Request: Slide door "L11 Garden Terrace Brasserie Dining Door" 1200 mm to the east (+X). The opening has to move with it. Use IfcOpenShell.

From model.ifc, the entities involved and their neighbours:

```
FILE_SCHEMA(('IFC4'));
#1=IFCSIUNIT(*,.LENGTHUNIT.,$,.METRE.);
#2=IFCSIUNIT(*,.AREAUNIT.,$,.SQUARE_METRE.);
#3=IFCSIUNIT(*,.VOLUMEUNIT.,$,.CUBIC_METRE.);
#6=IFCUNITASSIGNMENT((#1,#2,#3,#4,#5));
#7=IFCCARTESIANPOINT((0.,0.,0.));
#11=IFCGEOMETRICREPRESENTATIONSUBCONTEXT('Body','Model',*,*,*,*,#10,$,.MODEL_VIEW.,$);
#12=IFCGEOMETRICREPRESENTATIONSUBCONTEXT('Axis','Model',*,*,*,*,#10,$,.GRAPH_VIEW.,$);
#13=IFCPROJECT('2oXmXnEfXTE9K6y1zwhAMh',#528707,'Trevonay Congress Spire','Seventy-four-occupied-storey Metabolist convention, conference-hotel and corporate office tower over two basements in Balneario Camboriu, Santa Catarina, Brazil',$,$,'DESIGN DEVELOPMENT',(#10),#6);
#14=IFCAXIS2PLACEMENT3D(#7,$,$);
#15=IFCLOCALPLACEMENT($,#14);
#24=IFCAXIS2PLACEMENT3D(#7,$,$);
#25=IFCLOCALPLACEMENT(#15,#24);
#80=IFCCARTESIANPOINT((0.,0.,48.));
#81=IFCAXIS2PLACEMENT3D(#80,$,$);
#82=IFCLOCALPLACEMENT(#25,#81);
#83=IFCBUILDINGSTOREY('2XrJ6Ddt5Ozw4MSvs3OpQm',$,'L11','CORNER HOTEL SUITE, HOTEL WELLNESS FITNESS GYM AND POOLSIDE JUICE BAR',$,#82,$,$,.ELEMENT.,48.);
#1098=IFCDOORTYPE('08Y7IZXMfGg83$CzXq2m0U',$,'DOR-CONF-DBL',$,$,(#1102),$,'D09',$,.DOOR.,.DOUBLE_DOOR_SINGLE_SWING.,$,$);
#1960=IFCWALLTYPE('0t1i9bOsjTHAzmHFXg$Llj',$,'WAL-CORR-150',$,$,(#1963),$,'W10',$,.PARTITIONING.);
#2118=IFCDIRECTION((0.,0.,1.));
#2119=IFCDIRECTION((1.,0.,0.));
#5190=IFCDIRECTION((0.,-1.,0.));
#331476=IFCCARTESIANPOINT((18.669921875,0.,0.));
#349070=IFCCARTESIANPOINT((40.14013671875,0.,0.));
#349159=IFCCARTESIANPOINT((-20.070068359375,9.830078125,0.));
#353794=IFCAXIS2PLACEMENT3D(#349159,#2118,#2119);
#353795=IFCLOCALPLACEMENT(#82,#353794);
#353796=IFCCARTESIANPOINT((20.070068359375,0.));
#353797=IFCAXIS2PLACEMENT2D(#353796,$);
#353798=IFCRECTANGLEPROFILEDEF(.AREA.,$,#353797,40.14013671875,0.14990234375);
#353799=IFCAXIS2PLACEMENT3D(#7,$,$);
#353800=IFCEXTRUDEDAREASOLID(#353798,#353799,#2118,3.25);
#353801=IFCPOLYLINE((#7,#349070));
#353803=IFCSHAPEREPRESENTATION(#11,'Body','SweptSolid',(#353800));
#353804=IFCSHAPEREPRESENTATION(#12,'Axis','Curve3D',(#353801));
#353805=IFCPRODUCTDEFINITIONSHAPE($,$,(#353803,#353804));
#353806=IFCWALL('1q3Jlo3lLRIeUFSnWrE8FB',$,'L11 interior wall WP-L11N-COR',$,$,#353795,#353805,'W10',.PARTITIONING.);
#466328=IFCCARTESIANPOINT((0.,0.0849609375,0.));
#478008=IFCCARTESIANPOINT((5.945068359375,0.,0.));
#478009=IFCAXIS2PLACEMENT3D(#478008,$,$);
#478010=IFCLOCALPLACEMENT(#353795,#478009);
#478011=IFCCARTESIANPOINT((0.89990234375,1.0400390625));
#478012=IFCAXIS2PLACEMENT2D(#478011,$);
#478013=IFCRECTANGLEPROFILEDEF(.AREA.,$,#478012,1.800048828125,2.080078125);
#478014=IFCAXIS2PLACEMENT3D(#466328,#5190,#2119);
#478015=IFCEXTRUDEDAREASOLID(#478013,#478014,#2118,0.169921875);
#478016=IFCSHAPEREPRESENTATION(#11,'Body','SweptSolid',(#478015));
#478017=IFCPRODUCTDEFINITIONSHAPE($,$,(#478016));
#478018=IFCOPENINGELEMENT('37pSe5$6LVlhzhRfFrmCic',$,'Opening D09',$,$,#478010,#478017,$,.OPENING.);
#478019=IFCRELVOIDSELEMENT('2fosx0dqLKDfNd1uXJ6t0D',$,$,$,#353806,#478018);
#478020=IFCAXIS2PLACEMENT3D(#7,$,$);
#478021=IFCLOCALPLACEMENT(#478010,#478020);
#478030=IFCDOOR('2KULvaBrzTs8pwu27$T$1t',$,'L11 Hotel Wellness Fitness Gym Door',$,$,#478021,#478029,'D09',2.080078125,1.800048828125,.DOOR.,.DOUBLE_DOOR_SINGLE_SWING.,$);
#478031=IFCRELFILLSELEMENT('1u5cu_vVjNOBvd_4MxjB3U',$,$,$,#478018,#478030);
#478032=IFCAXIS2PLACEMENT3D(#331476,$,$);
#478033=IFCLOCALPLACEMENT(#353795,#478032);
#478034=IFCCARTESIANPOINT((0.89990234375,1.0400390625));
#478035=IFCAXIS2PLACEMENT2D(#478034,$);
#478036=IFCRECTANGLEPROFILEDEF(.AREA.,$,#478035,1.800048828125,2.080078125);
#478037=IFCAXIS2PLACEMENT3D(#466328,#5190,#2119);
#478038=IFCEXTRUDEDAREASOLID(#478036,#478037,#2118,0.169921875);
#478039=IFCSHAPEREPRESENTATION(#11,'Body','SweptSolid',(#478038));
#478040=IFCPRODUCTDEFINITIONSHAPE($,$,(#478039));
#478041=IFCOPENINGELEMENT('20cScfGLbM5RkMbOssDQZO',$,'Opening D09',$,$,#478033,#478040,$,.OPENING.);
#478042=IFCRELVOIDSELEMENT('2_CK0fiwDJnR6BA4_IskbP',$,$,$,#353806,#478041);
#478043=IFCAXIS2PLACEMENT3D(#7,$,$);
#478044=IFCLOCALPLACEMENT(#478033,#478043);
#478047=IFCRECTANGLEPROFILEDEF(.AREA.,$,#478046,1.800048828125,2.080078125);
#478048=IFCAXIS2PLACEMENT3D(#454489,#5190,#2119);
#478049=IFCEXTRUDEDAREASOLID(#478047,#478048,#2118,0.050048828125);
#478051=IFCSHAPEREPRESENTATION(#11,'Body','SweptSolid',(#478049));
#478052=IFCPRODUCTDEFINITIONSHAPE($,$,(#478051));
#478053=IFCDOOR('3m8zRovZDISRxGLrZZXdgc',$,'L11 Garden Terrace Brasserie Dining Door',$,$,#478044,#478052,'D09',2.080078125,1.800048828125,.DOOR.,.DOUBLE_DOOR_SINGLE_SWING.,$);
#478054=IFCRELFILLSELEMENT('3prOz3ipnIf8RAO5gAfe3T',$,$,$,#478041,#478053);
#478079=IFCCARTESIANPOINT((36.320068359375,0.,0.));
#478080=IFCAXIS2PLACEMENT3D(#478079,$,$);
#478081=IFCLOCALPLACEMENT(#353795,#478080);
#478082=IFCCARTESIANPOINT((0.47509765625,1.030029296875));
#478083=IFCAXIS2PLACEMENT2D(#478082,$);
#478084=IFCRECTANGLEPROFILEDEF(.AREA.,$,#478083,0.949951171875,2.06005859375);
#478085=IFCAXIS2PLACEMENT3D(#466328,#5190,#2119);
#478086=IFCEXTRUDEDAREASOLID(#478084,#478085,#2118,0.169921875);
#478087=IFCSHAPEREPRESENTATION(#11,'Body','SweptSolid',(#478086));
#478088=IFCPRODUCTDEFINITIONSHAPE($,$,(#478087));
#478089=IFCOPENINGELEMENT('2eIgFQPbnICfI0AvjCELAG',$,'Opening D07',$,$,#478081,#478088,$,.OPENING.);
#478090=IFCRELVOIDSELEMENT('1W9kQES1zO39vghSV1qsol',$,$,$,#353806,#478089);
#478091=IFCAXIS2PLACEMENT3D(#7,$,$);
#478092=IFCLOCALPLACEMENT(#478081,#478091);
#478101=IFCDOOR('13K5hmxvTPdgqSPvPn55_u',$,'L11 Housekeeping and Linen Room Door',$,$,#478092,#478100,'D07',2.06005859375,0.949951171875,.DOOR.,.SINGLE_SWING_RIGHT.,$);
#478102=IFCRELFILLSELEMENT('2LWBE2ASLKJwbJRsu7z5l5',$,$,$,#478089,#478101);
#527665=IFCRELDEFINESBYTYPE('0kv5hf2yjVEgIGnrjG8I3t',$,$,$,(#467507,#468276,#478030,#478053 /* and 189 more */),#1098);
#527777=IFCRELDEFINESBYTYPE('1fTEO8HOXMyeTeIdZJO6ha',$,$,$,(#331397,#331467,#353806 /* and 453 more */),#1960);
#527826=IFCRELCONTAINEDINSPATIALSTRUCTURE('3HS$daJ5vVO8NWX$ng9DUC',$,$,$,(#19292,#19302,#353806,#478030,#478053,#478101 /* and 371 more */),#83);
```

```python
import ifcopenshell
import ifcopenshell.api.geometry
import ifcopenshell.util.placement

model = ifcopenshell.open("model.ifc")

door = model.by_guid("3m8zRovZDISRxGLrZZXdgc")
opening = door.FillsVoids[0].RelatingOpeningElement
wall = opening.VoidsElements[0].RelatingBuildingElement

wall_matrix = ifcopenshell.util.placement.get_local_placement(wall.ObjectPlacement)
shift = wall_matrix[:3, 0] * 1.2
before = ifcopenshell.util.placement.get_local_placement(door.ObjectPlacement)[:3, 3].copy()

# The door is placed relative to its opening, so it follows when the opening moves.
matrix = ifcopenshell.util.placement.get_local_placement(opening.ObjectPlacement)
matrix[:3, 3] += shift
ifcopenshell.api.geometry.edit_object_placement(
    model, product=opening, matrix=matrix, is_si=False, should_transform_children=True
)

after = ifcopenshell.util.placement.get_local_placement(door.ObjectPlacement)[:3, 3]
print("door moved by", (after - before).round(3) + 0.0)

model.write("model_v2.ifc")
```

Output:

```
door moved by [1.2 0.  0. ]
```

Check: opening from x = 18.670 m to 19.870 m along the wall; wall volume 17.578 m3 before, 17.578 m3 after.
